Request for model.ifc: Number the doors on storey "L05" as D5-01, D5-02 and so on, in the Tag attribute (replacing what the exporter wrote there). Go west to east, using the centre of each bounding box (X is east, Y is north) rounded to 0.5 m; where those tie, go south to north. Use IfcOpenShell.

First a look at what the model holds.

```python
import ifcopenshell
import ifcopenshell.util.element
import ifcopenshell.util.placement

model = ifcopenshell.open("model.ifc")
print(model.schema)
storey = next(s for s in model.by_type("IfcBuildingStorey") if s.Name == "L05")
doors = [e for e in ifcopenshell.util.element.get_decomposition(storey) if e.is_a("IfcDoor")]
for e in sorted(doors, key=lambda e: e.id()):
    origin = ifcopenshell.util.placement.get_local_placement(e.ObjectPlacement)[:3, 3]
    print(e.id(), e.Tag, e.Name, origin.round(2) + 0.0, sep=" | ")
```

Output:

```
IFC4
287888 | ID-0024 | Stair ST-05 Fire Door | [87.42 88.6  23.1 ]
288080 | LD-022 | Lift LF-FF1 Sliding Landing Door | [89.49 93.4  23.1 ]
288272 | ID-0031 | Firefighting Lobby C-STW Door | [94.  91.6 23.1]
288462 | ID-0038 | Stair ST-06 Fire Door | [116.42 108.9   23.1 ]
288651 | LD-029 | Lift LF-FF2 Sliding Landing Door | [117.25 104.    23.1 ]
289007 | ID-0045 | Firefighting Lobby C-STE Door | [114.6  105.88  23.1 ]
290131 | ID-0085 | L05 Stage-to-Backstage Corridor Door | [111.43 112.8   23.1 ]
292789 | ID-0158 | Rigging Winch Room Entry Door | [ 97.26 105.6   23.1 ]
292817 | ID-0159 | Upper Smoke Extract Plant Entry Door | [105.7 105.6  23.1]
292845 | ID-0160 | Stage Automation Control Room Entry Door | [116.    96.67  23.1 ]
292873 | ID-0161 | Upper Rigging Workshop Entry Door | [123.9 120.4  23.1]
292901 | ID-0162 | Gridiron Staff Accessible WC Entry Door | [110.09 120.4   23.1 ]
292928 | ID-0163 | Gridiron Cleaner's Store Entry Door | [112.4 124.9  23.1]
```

```python
import ifcopenshell
import ifcopenshell.geom
import ifcopenshell.util.element
import ifcopenshell.util.shape

model = ifcopenshell.open("model.ifc")
settings = ifcopenshell.geom.settings()
settings.set("use-world-coords", True)


def centre(element):
    shape = ifcopenshell.geom.create_shape(settings, element)
    return ifcopenshell.util.shape.get_bbox_centroid(shape.geometry)


storey = next(s for s in model.by_type("IfcBuildingStorey") if s.Name == "L05")
doors = [e for e in ifcopenshell.util.element.get_decomposition(storey) if e.is_a("IfcDoor")]

# Insertion points can sit at a corner or the storey origin, so sort by the geometry (in metres).
centres = {e: centre(e) for e in doors}
doors.sort(key=lambda e: (round(centres[e][0] / 0.5), centres[e][1]))

for i, e in enumerate(doors, start=1):
    number = f"D5-{i:02d}"
    e.Tag = number
    print(e.id(), number)

model.write("model_v2.ifc")
```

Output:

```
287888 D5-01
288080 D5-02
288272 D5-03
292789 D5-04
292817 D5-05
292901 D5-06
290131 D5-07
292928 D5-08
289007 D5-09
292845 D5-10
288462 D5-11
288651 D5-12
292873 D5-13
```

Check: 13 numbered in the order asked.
